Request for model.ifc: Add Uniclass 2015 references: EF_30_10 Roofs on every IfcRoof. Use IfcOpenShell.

First a look at what the model holds.

```python
import ifcopenshell

model = ifcopenshell.open("model.ifc")
print(model.schema)
print("classifications:", [c.Name for c in model.by_type("IfcClassification")])
for ifc_class in ("IfcDoor", "IfcRoof", "IfcStair", "IfcWall", "IfcWindow"):
    print(ifc_class, len(model.by_type(ifc_class)))
```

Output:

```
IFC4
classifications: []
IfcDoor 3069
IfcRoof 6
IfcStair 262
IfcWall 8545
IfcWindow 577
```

```python
import ifcopenshell
import ifcopenshell.api.classification

model = ifcopenshell.open("model.ifc")

system = ifcopenshell.api.classification.add_classification(model, classification="Uniclass 2015")

codes = {
    "IfcRoof": ("EF_30_10", "Roofs"),
}
for ifc_class, (code, name) in codes.items():
    products = model.by_type(ifc_class)
    ifcopenshell.api.classification.add_reference(
        model, products=products, classification=system, identification=code, name=name
    )
    print(code, len(products))

model.write("model_v2.ifc")
```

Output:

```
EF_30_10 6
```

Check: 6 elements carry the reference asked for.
